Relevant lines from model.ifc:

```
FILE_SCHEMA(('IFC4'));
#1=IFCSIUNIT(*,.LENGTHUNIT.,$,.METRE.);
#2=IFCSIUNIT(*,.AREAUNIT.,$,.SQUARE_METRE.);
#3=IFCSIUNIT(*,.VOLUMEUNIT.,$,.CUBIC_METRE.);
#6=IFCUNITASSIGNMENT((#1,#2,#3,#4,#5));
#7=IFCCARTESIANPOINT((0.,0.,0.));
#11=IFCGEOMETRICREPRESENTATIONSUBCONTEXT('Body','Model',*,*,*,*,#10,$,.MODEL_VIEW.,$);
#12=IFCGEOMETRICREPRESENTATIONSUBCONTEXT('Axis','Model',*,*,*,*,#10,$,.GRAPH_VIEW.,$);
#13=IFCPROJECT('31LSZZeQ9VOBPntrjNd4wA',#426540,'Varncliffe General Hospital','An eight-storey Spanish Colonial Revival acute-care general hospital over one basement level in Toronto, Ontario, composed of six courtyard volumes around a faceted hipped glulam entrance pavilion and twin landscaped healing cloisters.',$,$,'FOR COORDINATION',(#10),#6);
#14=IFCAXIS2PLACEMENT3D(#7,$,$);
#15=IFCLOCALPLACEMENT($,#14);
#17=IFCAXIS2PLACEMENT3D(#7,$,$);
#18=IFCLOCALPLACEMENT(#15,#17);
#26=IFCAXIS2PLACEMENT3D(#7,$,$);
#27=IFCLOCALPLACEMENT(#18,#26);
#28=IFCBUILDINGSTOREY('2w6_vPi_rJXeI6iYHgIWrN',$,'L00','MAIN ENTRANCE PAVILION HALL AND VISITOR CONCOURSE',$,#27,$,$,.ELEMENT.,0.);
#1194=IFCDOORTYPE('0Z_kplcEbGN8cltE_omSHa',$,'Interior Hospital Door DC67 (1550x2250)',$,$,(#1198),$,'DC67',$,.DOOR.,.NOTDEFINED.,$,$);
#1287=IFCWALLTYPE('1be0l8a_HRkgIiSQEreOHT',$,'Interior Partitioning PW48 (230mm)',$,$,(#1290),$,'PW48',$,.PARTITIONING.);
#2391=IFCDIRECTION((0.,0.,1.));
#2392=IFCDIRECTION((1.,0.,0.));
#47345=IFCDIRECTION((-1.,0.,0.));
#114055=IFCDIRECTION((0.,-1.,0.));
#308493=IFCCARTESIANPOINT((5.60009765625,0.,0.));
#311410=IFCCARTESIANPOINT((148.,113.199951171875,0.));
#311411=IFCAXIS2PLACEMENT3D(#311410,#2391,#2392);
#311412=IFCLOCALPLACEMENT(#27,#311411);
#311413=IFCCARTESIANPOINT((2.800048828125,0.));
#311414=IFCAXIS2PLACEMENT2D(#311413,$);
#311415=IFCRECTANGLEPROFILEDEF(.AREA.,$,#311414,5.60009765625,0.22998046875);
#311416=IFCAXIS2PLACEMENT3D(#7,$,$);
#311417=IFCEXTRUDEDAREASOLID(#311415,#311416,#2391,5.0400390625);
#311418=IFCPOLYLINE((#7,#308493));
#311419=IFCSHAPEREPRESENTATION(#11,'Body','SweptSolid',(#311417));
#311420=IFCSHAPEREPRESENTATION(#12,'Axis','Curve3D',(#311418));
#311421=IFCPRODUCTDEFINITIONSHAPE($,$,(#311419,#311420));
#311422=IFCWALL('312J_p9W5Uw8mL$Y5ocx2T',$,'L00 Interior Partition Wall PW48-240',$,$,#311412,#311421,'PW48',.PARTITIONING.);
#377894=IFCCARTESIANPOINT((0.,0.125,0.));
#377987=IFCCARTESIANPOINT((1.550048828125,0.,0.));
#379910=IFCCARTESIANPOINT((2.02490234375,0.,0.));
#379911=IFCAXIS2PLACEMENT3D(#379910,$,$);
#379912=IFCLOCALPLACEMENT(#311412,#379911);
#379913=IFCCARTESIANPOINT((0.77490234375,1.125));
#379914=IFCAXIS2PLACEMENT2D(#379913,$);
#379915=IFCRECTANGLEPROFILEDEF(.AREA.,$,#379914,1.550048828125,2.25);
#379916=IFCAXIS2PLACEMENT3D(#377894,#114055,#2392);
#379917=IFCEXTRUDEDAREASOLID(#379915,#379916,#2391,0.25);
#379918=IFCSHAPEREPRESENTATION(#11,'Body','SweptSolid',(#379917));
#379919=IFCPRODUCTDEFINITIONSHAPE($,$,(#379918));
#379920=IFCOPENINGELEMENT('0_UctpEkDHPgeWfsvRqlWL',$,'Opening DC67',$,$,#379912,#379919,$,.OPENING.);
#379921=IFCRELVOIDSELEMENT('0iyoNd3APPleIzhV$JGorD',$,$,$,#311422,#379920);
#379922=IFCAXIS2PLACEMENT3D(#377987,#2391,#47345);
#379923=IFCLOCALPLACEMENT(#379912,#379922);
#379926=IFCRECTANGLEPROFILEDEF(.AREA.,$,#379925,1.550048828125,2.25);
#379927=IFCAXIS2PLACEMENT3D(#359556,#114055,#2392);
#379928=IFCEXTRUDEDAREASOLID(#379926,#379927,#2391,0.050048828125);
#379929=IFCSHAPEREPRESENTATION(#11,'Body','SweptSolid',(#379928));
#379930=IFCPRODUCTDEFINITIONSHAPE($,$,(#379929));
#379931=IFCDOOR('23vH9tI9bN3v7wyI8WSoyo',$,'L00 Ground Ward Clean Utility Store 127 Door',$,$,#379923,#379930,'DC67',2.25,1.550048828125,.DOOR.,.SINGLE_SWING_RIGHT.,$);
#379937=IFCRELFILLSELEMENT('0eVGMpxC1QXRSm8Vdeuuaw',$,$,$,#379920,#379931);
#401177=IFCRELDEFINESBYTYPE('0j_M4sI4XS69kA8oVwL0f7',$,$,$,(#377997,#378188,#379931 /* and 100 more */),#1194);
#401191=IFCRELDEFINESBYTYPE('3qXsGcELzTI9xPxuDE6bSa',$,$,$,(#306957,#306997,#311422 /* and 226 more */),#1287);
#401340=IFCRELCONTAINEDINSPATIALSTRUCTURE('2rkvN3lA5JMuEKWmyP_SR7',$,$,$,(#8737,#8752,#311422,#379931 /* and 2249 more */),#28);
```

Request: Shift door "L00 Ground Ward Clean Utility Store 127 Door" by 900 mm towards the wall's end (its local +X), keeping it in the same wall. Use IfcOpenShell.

```python
import ifcopenshell
import ifcopenshell.api.geometry
import ifcopenshell.util.placement
import ifcopenshell.util.unit

model = ifcopenshell.open("model.ifc")
unit_scale = ifcopenshell.util.unit.calculate_unit_scale(model)

door = model.by_guid("23vH9tI9bN3v7wyI8WSoyo")
opening = door.FillsVoids[0].RelatingOpeningElement
wall = opening.VoidsElements[0].RelatingBuildingElement

wall_matrix = ifcopenshell.util.placement.get_local_placement(wall.ObjectPlacement)
shift = wall_matrix[:3, 0] * 0.9 / unit_scale
before = ifcopenshell.util.placement.get_local_placement(door.ObjectPlacement)[:3, 3].copy()

# The door is placed relative to its opening, so it follows when the opening moves.
matrix = ifcopenshell.util.placement.get_local_placement(opening.ObjectPlacement)
matrix[:3, 3] += shift
ifcopenshell.api.geometry.edit_object_placement(
    model, product=opening, matrix=matrix, is_si=False, should_transform_children=True
)

after = ifcopenshell.util.placement.get_local_placement(door.ObjectPlacement)[:3, 3]
print("door moved by", (after - before).round(3) + 0.0)

model.write("model_edited.ifc")
```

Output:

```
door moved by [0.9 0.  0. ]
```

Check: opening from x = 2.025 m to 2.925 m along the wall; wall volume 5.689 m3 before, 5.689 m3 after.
